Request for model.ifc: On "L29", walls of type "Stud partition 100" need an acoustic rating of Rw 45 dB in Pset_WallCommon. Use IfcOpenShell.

First a look at what the model holds.

```python
import ifcopenshell
import ifcopenshell.util.element

model = ifcopenshell.open("model.ifc")
print(model.schema)
storey = next(s for s in model.by_type("IfcBuildingStorey") if s.Name == "L29")
walls = [e for e in ifcopenshell.util.element.get_decomposition(storey) if e.is_a("IfcWall")]
seen = {}
for e in walls:
    element_type = ifcopenshell.util.element.get_type(e)
    key = (element_type.Name if element_type != e and element_type else None, ifcopenshell.util.element.get_pset(e, "Pset_WallCommon", "AcousticRating"))
    seen[key] = seen.get(key, 0) + 1
for (name, value), count in sorted(seen.items(), key=str):
    print(count, "x", name, "|", value)
```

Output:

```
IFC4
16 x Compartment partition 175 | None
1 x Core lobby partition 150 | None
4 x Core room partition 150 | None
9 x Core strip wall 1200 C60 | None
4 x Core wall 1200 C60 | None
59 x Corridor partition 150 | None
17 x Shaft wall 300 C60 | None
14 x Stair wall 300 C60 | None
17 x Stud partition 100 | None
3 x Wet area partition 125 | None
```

```python
import ifcopenshell
import ifcopenshell.api.pset
import ifcopenshell.util.element

model = ifcopenshell.open("model.ifc")

storey = next(s for s in model.by_type("IfcBuildingStorey") if s.Name == "L29")
walls = [e for e in ifcopenshell.util.element.get_decomposition(storey) if e.is_a("IfcWall")]

count = 0
for e in walls:
    element_type = ifcopenshell.util.element.get_type(e)
    if element_type in (None, e) or element_type.Name != "Stud partition 100":
        continue
    found = ifcopenshell.util.element.get_pset(e, "Pset_WallCommon", should_inherit=False)
    if found:
        pset = model.by_id(found["id"])
        if len(ifcopenshell.util.element.get_elements_by_pset(pset)) > 1:
            pset = ifcopenshell.api.pset.unshare_pset(model, products=[e], pset=pset)[0]
    else:
        pset = ifcopenshell.api.pset.add_pset(model, product=e, name="Pset_WallCommon")
    ifcopenshell.api.pset.edit_pset(model, pset=pset, properties={"AcousticRating": "Rw 45 dB"})
    count += 1

print(count, "walls updated")

model.write("model_rev.ifc")
```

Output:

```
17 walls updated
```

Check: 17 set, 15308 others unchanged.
